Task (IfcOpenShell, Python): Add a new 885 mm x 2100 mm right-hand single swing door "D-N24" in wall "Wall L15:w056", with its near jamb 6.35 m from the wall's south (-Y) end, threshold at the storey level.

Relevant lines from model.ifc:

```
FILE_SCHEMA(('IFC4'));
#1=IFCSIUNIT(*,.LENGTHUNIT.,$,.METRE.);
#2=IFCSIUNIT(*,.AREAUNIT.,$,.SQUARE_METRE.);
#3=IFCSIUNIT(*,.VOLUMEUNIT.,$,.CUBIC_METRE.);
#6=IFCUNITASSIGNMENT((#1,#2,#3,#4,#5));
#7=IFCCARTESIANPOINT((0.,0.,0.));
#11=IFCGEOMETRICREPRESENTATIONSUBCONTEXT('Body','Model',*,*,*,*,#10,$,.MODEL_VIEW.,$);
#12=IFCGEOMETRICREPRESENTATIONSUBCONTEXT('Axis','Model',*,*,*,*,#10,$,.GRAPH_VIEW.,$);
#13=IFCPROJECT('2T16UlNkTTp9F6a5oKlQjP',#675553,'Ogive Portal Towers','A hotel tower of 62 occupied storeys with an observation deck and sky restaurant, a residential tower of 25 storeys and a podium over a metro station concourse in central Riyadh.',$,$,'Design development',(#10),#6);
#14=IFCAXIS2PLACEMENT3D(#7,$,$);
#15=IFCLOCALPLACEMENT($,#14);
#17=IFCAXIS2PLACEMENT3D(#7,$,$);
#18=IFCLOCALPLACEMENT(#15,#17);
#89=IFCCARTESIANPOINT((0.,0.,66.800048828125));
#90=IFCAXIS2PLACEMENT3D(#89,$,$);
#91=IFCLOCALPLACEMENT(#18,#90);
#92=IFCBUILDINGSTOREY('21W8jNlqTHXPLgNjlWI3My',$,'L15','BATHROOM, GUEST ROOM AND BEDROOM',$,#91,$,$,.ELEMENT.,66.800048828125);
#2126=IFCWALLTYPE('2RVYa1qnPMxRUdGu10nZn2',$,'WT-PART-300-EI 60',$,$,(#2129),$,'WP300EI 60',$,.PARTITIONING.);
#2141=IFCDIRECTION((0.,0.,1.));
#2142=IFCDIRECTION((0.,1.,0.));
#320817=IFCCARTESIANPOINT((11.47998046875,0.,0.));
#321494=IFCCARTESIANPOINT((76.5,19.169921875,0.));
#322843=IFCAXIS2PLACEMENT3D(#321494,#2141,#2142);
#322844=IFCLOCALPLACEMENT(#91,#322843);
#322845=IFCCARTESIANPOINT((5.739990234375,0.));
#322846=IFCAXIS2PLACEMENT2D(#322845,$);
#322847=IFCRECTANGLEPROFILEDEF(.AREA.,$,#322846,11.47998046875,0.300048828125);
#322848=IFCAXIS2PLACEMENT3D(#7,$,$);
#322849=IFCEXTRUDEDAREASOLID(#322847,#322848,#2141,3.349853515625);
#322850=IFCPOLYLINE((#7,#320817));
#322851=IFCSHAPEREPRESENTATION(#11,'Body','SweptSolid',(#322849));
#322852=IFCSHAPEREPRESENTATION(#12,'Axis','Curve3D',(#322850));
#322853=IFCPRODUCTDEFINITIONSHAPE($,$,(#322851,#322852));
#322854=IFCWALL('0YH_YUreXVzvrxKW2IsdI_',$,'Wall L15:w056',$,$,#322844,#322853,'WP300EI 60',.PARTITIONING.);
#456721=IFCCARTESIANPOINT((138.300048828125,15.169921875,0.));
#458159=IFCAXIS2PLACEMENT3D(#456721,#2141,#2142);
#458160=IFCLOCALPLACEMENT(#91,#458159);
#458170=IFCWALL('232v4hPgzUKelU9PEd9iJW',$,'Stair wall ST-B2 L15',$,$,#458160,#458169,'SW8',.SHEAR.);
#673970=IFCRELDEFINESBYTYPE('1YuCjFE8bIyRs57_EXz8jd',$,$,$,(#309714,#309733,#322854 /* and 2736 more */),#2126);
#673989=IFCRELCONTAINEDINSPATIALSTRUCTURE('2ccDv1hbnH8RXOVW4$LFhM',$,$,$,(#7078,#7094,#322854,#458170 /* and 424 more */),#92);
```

```python
import numpy as np
import ifcopenshell
import ifcopenshell.api.feature
import ifcopenshell.api.geometry
import ifcopenshell.api.root
import ifcopenshell.api.spatial
import ifcopenshell.geom
import ifcopenshell.util.element
import ifcopenshell.util.placement
import ifcopenshell.util.representation
import ifcopenshell.util.shape
import ifcopenshell.util.unit

model = ifcopenshell.open("model.ifc")
unit_scale = ifcopenshell.util.unit.calculate_unit_scale(model)
settings = ifcopenshell.geom.settings()


def volume(element):
    """Net volume in cubic metres, openings subtracted."""
    shape = ifcopenshell.geom.create_shape(settings, element)
    return ifcopenshell.util.shape.get_volume(shape.geometry)


wall = model.by_guid("0YH_YUreXVzvrxKW2IsdI_")
storey = ifcopenshell.util.element.get_container(wall, ifc_class="IfcBuildingStorey")
context = ifcopenshell.util.representation.get_context(model, "Model", "Body", "MODEL_VIEW")
before = volume(wall)

width, height, from_end, sill = 0.885, 2.1, 6.35, 0.0  # metres

# The wall runs along its own X axis, and the end named is its -X end.
wall_shape = ifcopenshell.geom.create_shape(settings, wall)
x, y, z = ifcopenshell.util.shape.get_vertices(wall_shape.geometry).T
start = x.min() + from_end
face, thickness = float(y.min()), float(y.max() - y.min())
wall_matrix = ifcopenshell.util.placement.get_local_placement(wall.ObjectPlacement)
level = ifcopenshell.util.placement.get_local_placement(storey.ObjectPlacement)[2, 3]


def in_wall(x, y):
    """Placement at x, y metres in the wall's axes, at sill height."""
    matrix = wall_matrix.copy()
    matrix[:, 3] = wall_matrix @ np.array([x / unit_scale, y / unit_scale, 0.0, 1.0])
    matrix[2, 3] = level + sill / unit_scale
    return matrix


# Opening: a box that overshoots both wall faces by 50 mm.
opening = ifcopenshell.api.root.create_entity(model, ifc_class="IfcOpeningElement", predefined_type="OPENING")
box = ifcopenshell.api.geometry.add_wall_representation(
    model, context=context, length=width, height=height, thickness=thickness + 0.1
)
ifcopenshell.api.geometry.assign_representation(model, product=opening, representation=box)
ifcopenshell.api.geometry.edit_object_placement(model, product=opening, matrix=in_wall(start, face - 0.05), is_si=False)
ifcopenshell.api.feature.add_feature(model, feature=opening, element=wall)

door = ifcopenshell.api.root.create_entity(model, ifc_class="IfcDoor", name="D-N24", predefined_type="DOOR")
door.OverallWidth, door.OverallHeight = width / unit_scale, height / unit_scale
door.OperationType = "SINGLE_SWING_RIGHT"
body = ifcopenshell.api.geometry.add_door_representation(
    model,
    context=context,
    overall_width=door.OverallWidth,
    overall_height=door.OverallHeight,
    operation_type="SINGLE_SWING_RIGHT",
    lining_properties={"LiningDepth": thickness / unit_scale, "ThresholdDepth": thickness / unit_scale},
)
ifcopenshell.api.geometry.assign_representation(model, product=door, representation=body)
ifcopenshell.api.spatial.assign_container(model, products=[door], relating_structure=storey)
ifcopenshell.api.feature.add_filling(model, opening=opening, element=door)

# The lining spans the wall, so the door starts at the wall face.
ifcopenshell.api.geometry.edit_object_placement(model, product=door, matrix=in_wall(start, face), is_si=False)

after = volume(wall)

print(f"wall volume {before:.3f} -> {after:.3f} m3")

model.write("model_updated.ifc")
```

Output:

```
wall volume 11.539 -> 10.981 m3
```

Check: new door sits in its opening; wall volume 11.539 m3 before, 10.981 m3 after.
